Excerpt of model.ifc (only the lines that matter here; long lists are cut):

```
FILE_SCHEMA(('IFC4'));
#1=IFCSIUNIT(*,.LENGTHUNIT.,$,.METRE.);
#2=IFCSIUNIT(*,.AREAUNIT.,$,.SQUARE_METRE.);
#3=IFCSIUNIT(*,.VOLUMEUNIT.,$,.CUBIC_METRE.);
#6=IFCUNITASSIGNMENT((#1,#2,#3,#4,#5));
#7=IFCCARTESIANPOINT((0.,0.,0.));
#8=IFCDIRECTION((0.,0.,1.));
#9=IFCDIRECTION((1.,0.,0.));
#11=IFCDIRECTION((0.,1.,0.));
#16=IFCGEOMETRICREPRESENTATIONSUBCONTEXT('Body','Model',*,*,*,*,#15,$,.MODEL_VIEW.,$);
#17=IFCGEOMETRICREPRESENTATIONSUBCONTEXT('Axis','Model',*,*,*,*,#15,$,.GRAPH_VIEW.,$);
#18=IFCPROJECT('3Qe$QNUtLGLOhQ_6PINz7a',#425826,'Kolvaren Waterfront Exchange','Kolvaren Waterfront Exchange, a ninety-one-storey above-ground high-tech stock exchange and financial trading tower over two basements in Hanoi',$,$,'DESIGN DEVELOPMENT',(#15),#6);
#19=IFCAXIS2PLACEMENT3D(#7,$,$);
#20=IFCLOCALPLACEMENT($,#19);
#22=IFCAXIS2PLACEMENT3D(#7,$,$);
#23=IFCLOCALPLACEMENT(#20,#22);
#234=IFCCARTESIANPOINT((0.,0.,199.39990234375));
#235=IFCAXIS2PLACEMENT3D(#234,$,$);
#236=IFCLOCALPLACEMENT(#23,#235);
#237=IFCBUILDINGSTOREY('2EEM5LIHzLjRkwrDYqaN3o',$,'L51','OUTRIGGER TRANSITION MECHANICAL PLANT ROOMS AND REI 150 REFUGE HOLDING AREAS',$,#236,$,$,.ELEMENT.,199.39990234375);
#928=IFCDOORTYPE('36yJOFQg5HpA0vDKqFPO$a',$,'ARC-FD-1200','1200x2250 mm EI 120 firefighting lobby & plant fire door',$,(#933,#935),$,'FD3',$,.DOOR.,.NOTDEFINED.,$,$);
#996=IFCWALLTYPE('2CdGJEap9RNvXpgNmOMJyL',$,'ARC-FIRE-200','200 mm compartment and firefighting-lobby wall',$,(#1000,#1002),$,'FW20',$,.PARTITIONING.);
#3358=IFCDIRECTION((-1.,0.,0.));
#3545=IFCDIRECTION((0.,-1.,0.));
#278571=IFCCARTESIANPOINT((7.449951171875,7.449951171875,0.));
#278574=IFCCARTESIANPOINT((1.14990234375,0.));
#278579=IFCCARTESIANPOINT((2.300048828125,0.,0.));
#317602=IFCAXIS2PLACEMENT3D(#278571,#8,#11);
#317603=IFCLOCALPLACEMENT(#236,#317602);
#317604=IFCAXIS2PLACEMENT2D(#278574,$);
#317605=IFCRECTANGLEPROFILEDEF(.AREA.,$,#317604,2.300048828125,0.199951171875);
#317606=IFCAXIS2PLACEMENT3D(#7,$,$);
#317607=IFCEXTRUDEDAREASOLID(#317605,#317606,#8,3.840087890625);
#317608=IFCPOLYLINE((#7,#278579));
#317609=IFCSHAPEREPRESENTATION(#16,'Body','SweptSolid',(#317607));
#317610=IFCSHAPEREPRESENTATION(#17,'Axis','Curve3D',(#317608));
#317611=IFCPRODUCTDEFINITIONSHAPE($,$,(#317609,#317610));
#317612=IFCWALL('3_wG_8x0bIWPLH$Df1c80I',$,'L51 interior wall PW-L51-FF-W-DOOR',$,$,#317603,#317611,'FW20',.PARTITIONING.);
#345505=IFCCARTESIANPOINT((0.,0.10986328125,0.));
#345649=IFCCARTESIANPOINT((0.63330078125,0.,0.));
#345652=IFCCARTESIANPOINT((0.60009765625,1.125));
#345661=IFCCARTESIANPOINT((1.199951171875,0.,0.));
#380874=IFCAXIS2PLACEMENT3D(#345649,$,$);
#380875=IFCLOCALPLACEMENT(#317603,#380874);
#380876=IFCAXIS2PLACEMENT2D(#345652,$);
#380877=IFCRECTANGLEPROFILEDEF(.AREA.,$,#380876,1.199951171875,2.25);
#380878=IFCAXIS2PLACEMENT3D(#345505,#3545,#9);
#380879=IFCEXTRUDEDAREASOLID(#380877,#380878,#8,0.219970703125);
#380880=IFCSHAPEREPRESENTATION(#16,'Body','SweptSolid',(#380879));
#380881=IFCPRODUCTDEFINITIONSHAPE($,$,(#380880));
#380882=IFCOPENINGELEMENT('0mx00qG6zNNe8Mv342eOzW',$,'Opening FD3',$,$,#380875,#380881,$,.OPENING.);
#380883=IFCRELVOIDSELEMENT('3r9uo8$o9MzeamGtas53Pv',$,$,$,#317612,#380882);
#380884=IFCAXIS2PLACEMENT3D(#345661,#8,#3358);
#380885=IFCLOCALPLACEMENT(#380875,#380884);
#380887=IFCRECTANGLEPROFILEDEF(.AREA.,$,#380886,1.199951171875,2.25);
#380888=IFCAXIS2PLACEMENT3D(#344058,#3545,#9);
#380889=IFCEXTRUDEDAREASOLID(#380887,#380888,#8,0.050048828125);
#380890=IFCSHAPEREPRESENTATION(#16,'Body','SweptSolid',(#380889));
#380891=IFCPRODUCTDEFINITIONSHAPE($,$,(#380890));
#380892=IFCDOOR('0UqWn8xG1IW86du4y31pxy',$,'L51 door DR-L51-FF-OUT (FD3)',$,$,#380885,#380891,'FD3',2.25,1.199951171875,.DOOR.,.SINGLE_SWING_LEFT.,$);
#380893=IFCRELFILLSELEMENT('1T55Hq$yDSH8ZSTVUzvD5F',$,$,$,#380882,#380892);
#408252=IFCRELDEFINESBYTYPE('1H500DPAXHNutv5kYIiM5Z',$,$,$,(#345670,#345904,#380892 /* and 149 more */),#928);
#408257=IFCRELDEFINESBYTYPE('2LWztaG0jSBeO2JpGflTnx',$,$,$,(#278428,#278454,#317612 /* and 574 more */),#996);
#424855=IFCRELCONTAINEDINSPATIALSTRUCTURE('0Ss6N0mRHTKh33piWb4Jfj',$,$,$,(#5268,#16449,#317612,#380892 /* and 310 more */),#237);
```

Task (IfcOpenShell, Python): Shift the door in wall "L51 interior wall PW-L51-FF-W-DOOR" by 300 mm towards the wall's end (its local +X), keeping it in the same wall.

```python
import ifcopenshell
import ifcopenshell.api.geometry
import ifcopenshell.util.placement
import ifcopenshell.util.unit

model = ifcopenshell.open("model.ifc")
unit_scale = ifcopenshell.util.unit.calculate_unit_scale(model)

door = model.by_guid("0UqWn8xG1IW86du4y31pxy")
opening = door.FillsVoids[0].RelatingOpeningElement
wall = opening.VoidsElements[0].RelatingBuildingElement

wall_matrix = ifcopenshell.util.placement.get_local_placement(wall.ObjectPlacement)
shift = wall_matrix[:3, 0] * 0.3 / unit_scale
before = ifcopenshell.util.placement.get_local_placement(door.ObjectPlacement)[:3, 3].copy()

# The door is placed relative to its opening, so it follows when the opening moves.
matrix = ifcopenshell.util.placement.get_local_placement(opening.ObjectPlacement)
matrix[:3, 3] += shift
ifcopenshell.api.geometry.edit_object_placement(
    model, product=opening, matrix=matrix, is_si=False, should_transform_children=True
)

after = ifcopenshell.util.placement.get_local_placement(door.ObjectPlacement)[:3, 3]
print("door moved by", (after - before).round(3) + 0.0)

model.write("model_edited.ifc")
```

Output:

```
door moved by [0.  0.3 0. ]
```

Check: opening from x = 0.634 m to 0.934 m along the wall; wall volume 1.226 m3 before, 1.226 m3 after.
